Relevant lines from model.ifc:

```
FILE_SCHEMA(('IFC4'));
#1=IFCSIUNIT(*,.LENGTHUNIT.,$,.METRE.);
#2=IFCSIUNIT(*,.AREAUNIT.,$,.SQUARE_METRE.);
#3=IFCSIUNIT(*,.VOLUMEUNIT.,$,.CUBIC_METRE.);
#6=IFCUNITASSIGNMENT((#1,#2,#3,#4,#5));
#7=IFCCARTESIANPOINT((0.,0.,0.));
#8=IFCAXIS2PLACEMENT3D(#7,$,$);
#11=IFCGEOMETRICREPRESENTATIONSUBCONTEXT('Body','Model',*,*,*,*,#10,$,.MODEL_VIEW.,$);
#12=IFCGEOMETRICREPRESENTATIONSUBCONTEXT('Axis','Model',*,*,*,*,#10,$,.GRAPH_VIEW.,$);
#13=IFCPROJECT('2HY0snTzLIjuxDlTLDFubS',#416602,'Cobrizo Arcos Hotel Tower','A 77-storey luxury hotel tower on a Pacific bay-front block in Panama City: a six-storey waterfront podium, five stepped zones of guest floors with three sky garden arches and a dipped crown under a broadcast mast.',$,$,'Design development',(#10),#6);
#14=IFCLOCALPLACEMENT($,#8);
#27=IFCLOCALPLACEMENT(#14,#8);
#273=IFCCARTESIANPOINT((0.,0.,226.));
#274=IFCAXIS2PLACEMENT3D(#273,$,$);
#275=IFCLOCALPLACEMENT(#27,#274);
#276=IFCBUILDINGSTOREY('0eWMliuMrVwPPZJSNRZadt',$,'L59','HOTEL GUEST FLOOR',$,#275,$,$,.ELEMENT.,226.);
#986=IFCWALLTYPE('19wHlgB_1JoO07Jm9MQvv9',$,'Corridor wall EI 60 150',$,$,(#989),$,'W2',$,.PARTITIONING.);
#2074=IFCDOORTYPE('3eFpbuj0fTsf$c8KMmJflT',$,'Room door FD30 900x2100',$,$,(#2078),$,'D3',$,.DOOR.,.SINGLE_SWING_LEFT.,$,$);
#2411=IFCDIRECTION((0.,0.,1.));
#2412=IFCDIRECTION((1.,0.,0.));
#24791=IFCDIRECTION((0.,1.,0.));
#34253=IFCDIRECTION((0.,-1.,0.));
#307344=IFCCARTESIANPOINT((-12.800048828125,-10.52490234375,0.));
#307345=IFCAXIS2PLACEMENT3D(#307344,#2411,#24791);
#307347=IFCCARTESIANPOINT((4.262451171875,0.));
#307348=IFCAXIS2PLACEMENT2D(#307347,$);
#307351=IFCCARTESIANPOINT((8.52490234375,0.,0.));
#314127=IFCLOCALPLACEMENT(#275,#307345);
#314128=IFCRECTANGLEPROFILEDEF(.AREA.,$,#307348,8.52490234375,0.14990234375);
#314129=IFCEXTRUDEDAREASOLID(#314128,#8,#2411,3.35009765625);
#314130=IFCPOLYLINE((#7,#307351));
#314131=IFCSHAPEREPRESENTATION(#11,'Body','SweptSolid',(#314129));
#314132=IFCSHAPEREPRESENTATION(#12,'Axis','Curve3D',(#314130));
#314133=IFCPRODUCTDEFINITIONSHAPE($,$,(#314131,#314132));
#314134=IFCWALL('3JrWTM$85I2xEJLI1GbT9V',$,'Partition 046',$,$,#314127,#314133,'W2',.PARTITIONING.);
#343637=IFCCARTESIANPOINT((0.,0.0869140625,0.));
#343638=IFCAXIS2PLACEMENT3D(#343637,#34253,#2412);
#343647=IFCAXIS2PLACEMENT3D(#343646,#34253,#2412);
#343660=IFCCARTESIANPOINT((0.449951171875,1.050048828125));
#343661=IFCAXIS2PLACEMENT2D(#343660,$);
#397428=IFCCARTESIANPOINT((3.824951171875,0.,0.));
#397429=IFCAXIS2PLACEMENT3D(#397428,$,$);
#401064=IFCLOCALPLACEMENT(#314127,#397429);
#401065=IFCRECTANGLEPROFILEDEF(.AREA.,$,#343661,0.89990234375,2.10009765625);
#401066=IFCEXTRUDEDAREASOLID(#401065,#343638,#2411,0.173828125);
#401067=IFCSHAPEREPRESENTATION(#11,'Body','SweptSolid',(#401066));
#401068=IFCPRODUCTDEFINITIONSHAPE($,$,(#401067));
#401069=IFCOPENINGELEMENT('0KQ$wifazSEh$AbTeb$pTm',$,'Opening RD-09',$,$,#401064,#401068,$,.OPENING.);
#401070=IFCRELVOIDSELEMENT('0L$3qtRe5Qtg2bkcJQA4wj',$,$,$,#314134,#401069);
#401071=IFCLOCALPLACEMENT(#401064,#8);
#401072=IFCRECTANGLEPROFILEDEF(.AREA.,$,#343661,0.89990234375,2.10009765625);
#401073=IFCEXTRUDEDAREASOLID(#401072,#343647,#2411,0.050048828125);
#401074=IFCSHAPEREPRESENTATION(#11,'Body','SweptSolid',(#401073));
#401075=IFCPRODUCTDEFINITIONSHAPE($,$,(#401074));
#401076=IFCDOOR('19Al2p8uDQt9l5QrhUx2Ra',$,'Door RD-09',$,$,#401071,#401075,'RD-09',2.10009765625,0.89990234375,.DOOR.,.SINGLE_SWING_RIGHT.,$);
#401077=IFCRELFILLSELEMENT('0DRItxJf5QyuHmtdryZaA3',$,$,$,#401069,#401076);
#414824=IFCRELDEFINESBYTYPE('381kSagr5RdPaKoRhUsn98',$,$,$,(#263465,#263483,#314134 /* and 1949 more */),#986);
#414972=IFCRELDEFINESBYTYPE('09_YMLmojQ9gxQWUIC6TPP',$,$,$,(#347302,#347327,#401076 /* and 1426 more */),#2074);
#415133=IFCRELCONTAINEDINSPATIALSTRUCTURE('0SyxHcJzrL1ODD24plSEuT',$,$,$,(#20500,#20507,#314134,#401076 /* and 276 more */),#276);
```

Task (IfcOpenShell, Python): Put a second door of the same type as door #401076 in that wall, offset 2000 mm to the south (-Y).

```python
import ifcopenshell
import ifcopenshell.api.feature
import ifcopenshell.api.geometry
import ifcopenshell.api.root
import ifcopenshell.geom
import ifcopenshell.util.element
import ifcopenshell.util.placement
import ifcopenshell.util.shape
import ifcopenshell.util.unit

model = ifcopenshell.open("model.ifc")
unit_scale = ifcopenshell.util.unit.calculate_unit_scale(model)
settings = ifcopenshell.geom.settings()


def volume(element):
    """Net volume in cubic metres, openings subtracted."""
    shape = ifcopenshell.geom.create_shape(settings, element)
    return ifcopenshell.util.shape.get_volume(shape.geometry)


door = model.by_guid("19Al2p8uDQt9l5QrhUx2Ra")
opening = door.FillsVoids[0].RelatingOpeningElement
wall = opening.VoidsElements[0].RelatingBuildingElement
before = volume(wall)
shift = ifcopenshell.util.placement.get_local_placement(wall.ObjectPlacement)[:3, 0] * -2 / unit_scale

# copy_class copies the void relationship, type, container and properties, but no geometry.
new_opening = ifcopenshell.api.root.copy_class(model, product=opening)
new_opening.Representation = ifcopenshell.util.element.copy_deep(
    model, opening.Representation, exclude=["IfcGeometricRepresentationContext", "IfcRepresentationMap"]
)
new_door = ifcopenshell.api.root.copy_class(model, product=door)
new_door.Representation = ifcopenshell.util.element.copy_deep(
    model, door.Representation, exclude=["IfcGeometricRepresentationContext", "IfcRepresentationMap"]
)
new_door.Tag = None
ifcopenshell.api.feature.add_filling(model, opening=new_opening, element=new_door)

for old, new in ((opening, new_opening), (door, new_door)):
    matrix = ifcopenshell.util.placement.get_local_placement(old.ObjectPlacement)
    matrix[:3, 3] += shift
    ifcopenshell.api.geometry.edit_object_placement(model, product=new, matrix=matrix, is_si=False)

after = volume(wall)

print(f"wall volume {before:.3f} -> {after:.3f} m3")

model.write("model_v2.ifc")
```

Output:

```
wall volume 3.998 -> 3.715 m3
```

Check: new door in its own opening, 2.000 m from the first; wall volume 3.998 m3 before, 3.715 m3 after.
